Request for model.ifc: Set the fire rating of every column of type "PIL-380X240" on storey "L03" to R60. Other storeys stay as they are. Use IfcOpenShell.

First a look at what the model holds.

```python
import ifcopenshell
import ifcopenshell.util.element

model = ifcopenshell.open("model.ifc")
print(model.schema)
storey = next(s for s in model.by_type("IfcBuildingStorey") if s.Name == "L03")
columns = [e for e in ifcopenshell.util.element.get_decomposition(storey) if e.is_a("IfcColumn")]
seen = {}
for e in columns:
    element_type = ifcopenshell.util.element.get_type(e)
    key = (element_type.Name if element_type != e and element_type else None, ifcopenshell.util.element.get_pset(e, "Pset_ColumnCommon", "FireRating"))
    seen[key] = seen.get(key, 0) + 1
for (name, value), count in sorted(seen.items(), key=str):
    print(count, "x", name, "|", value)
```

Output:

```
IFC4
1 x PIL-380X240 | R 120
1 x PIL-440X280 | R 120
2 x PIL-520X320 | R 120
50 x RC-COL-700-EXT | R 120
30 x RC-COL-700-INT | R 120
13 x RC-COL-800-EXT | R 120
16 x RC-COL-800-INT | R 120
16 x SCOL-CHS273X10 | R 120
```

```python
import ifcopenshell
import ifcopenshell.api.pset
import ifcopenshell.util.element

model = ifcopenshell.open("model.ifc")

storey = next(s for s in model.by_type("IfcBuildingStorey") if s.Name == "L03")
columns = [e for e in ifcopenshell.util.element.get_decomposition(storey) if e.is_a("IfcColumn")]

count = 0
for e in columns:
    element_type = ifcopenshell.util.element.get_type(e)
    if element_type in (None, e) or element_type.Name != "PIL-380X240":
        continue
    # add_pset returns the element's existing set when there is one.
    pset = ifcopenshell.api.pset.add_pset(model, product=e, name="Pset_ColumnCommon")
    ifcopenshell.api.pset.edit_pset(model, pset=pset, properties={"FireRating": "R60"})
    count += 1

print(count, "columns updated")

model.write("model_rev.ifc")
```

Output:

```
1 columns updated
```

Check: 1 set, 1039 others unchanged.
